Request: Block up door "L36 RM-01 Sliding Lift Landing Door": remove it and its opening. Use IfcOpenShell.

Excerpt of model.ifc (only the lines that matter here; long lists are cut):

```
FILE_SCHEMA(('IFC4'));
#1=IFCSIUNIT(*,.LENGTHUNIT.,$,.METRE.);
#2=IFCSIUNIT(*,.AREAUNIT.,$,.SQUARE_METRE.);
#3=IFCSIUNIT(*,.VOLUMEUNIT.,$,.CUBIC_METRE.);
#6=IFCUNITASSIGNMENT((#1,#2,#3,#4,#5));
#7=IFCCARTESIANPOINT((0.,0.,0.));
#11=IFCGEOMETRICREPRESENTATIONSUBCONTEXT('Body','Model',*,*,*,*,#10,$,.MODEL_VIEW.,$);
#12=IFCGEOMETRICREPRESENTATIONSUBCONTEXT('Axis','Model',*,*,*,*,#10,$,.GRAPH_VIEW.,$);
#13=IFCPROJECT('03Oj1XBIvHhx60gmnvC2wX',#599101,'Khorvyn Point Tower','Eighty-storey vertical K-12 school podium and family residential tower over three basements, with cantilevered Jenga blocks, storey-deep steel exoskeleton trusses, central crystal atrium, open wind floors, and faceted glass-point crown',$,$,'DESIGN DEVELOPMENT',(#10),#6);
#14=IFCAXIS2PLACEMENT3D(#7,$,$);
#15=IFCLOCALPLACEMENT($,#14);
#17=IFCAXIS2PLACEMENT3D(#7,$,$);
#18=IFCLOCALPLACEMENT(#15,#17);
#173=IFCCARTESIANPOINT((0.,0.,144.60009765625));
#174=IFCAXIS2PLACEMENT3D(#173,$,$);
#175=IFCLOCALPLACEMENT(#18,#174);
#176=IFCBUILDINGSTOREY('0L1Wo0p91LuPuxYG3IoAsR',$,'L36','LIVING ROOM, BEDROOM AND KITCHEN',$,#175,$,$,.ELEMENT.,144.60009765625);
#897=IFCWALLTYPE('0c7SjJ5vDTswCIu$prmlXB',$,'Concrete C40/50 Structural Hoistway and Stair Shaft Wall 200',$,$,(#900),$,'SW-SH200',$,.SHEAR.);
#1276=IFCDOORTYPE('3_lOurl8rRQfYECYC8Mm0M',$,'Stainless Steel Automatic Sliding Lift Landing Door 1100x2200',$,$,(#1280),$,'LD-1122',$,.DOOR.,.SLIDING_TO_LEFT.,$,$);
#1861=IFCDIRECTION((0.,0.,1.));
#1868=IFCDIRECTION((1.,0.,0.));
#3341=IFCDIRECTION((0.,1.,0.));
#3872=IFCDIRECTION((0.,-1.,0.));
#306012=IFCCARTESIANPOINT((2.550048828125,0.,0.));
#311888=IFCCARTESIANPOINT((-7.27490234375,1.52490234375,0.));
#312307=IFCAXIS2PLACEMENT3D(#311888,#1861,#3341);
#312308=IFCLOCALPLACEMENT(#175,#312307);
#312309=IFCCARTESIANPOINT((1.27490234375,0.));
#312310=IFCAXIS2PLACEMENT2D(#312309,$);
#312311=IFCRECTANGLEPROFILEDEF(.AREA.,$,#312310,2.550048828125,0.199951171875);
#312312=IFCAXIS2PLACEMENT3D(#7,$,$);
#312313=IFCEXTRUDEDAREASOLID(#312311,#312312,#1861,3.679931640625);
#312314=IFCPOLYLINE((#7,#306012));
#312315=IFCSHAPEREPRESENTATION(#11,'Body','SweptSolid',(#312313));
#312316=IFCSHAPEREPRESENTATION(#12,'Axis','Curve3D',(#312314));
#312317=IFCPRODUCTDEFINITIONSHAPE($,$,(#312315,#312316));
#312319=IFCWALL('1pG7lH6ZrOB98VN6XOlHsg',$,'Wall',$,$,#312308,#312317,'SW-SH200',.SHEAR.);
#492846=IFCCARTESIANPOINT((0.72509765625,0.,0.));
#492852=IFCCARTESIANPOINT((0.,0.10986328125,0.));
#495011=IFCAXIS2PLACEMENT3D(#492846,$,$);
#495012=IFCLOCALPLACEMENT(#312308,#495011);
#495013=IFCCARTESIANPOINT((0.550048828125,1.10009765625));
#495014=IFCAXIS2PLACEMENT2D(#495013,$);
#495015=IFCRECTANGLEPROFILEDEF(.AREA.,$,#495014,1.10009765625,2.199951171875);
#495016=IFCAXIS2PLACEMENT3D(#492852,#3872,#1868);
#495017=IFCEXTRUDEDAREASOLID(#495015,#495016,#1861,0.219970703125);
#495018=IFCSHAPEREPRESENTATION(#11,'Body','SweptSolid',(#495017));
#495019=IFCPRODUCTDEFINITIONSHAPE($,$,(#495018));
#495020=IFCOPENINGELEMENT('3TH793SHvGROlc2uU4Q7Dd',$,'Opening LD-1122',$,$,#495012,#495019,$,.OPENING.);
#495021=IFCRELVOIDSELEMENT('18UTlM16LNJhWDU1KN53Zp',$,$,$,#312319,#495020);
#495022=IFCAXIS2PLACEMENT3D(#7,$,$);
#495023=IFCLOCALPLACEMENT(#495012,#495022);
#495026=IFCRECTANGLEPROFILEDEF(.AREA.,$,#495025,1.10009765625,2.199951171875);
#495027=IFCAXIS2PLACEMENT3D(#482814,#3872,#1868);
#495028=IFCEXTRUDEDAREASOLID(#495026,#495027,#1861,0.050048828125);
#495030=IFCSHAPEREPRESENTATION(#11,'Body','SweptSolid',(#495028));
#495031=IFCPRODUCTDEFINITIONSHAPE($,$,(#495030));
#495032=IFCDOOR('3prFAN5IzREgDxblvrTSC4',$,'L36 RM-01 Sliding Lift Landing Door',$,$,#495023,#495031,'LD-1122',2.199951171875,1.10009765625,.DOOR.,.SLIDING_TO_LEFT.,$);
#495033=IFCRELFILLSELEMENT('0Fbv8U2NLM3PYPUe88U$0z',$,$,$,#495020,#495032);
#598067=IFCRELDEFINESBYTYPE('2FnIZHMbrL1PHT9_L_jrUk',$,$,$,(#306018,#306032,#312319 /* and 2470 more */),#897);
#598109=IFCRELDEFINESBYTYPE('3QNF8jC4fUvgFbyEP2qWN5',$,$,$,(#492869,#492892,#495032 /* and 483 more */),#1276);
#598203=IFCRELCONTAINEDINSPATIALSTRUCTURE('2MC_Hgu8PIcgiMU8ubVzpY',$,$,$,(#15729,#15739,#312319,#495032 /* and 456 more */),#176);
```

```python
import ifcopenshell
import ifcopenshell.api.feature
import ifcopenshell.api.root
import ifcopenshell.geom
import ifcopenshell.util.shape

model = ifcopenshell.open("model.ifc")
settings = ifcopenshell.geom.settings()


def volume(element):
    """Net volume in cubic metres, openings subtracted."""
    shape = ifcopenshell.geom.create_shape(settings, element)
    return ifcopenshell.util.shape.get_volume(shape.geometry)


door = model.by_guid("3prFAN5IzREgDxblvrTSC4")
opening = door.FillsVoids[0].RelatingOpeningElement
wall = opening.VoidsElements[0].RelatingBuildingElement
before = volume(wall)

ifcopenshell.api.root.remove_product(model, product=door)
ifcopenshell.api.feature.remove_feature(model, feature=opening)

after = volume(wall)

print(f"wall volume {before:.3f} -> {after:.3f} m3")

model.write("model_edited.ifc")
```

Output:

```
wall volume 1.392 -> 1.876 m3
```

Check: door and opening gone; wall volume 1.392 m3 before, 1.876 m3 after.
